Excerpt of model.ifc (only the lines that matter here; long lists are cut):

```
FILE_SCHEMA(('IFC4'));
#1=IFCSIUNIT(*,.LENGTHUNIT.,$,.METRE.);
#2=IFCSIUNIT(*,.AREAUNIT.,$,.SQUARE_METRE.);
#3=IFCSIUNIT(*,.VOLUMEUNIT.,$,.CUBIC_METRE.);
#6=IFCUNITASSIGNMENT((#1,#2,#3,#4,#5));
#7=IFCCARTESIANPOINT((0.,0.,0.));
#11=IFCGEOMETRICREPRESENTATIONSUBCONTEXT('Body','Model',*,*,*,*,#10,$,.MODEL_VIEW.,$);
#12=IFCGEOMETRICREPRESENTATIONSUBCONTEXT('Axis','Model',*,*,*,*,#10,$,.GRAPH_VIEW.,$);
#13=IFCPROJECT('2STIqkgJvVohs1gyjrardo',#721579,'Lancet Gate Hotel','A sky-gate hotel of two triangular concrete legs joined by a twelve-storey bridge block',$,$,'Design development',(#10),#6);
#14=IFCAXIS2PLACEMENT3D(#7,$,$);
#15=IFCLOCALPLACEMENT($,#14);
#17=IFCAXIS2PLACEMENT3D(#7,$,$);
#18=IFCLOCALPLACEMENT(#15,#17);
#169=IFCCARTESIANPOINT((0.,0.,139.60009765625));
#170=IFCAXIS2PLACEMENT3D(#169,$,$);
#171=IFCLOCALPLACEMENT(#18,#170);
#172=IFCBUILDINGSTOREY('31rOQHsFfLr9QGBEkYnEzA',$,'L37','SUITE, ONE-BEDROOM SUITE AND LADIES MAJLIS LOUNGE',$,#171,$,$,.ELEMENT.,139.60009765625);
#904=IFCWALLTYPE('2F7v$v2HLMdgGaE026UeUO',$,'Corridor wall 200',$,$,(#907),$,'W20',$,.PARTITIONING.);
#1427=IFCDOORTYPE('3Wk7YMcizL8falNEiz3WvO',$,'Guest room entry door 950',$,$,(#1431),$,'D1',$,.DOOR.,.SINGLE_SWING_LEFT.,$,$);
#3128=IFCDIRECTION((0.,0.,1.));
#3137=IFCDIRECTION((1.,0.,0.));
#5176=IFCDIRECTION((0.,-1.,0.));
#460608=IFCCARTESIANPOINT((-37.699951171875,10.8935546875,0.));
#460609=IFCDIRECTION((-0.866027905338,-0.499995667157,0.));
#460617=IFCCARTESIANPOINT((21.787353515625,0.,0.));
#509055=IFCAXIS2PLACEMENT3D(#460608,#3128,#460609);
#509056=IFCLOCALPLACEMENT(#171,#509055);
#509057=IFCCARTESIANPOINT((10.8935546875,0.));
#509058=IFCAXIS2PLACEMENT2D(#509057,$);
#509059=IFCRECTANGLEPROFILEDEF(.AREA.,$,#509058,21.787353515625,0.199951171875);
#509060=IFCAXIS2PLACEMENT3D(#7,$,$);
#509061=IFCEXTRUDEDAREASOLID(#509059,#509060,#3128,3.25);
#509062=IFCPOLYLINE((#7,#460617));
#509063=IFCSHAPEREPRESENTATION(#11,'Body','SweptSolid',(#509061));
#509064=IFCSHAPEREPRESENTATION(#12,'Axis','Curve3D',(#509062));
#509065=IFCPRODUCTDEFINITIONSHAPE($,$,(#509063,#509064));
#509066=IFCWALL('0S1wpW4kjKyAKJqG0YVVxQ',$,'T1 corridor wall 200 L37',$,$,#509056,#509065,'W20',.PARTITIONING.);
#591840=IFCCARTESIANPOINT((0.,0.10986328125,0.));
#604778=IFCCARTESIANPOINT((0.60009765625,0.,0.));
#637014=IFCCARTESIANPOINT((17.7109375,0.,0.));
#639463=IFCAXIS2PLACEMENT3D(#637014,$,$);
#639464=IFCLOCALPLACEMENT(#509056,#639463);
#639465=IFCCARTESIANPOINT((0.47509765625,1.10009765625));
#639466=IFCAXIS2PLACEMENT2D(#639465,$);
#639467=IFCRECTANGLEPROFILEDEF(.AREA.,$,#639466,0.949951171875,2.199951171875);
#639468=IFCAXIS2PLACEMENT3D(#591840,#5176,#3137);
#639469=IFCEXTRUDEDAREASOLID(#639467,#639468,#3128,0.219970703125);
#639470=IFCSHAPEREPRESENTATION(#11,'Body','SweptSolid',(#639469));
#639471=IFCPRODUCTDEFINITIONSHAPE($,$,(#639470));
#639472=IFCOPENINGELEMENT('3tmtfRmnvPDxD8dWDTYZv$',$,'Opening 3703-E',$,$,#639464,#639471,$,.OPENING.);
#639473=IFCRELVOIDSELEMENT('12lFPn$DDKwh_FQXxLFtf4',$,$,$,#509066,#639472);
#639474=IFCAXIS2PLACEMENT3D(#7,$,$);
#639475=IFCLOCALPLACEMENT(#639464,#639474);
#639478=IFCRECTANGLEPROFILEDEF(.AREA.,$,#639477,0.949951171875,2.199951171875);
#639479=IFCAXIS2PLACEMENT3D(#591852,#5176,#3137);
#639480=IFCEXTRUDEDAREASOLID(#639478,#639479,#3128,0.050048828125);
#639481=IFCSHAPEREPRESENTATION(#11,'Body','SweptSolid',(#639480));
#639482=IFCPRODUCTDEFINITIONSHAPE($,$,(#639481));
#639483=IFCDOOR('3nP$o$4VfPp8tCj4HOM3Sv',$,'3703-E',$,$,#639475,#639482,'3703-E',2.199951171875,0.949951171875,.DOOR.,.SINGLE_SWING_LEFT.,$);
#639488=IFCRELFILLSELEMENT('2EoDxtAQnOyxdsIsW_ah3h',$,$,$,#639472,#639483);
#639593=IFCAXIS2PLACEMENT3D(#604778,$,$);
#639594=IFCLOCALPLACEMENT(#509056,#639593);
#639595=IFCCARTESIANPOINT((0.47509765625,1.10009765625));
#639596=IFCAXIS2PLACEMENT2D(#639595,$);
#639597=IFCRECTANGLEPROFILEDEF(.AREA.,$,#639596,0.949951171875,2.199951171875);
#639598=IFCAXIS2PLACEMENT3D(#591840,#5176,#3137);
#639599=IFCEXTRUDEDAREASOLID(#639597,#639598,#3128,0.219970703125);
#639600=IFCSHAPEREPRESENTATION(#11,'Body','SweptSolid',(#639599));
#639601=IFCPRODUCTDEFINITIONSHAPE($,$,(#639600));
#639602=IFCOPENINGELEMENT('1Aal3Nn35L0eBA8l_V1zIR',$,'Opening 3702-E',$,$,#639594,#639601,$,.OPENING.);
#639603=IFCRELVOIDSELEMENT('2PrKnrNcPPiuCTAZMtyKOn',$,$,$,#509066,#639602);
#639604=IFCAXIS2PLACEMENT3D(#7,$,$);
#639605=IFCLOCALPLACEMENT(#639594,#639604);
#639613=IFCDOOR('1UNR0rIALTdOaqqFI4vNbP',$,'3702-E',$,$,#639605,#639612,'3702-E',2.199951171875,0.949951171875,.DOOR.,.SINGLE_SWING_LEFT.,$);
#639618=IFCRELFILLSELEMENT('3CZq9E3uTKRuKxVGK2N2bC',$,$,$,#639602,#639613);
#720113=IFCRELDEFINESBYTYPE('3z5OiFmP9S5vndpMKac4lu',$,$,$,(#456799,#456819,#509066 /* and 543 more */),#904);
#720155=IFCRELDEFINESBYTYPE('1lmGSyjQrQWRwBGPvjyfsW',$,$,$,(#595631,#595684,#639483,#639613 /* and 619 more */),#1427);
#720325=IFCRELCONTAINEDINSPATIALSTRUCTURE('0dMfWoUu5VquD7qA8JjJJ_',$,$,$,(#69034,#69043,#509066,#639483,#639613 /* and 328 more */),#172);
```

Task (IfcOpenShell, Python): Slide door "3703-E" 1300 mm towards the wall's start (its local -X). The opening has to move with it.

```python
import ifcopenshell
import ifcopenshell.api.geometry
import ifcopenshell.util.placement
import ifcopenshell.util.unit

model = ifcopenshell.open("model.ifc")
unit_scale = ifcopenshell.util.unit.calculate_unit_scale(model)

door = model.by_guid("3nP$o$4VfPp8tCj4HOM3Sv")
opening = door.FillsVoids[0].RelatingOpeningElement
wall = opening.VoidsElements[0].RelatingBuildingElement

wall_matrix = ifcopenshell.util.placement.get_local_placement(wall.ObjectPlacement)
shift = wall_matrix[:3, 0] * -1.3 / unit_scale
before = ifcopenshell.util.placement.get_local_placement(door.ObjectPlacement)[:3, 3].copy()

# The door is placed relative to its opening, so it follows when the opening moves.
matrix = ifcopenshell.util.placement.get_local_placement(opening.ObjectPlacement)
matrix[:3, 3] += shift
ifcopenshell.api.geometry.edit_object_placement(
    model, product=opening, matrix=matrix, is_si=False, should_transform_children=True
)

after = ifcopenshell.util.placement.get_local_placement(door.ObjectPlacement)[:3, 3]
print("door moved by", (after - before).round(3) + 0.0)

model.write("model_v2.ifc")
```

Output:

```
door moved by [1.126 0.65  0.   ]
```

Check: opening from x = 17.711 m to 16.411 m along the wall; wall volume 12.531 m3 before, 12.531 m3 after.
